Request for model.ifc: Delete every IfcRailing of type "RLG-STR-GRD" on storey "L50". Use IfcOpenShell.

First a look at what the model holds.

```python
import ifcopenshell
import ifcopenshell.util.element

model = ifcopenshell.open("model.ifc")
print(model.schema)
storey = next(s for s in model.by_type("IfcBuildingStorey") if s.Name == "L50")
railings = [e for e in ifcopenshell.util.element.get_decomposition(storey) if e.is_a("IfcRailing")]
seen = {}
for e in railings:
    element_type = ifcopenshell.util.element.get_type(e)
    name = element_type.Name if element_type not in (None, e) else None
    seen[name] = seen.get(name, 0) + 1
for name, count in sorted(seen.items(), key=str):
    print(count, "x", name)
```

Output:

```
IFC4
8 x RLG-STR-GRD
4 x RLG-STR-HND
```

```python
import ifcopenshell
import ifcopenshell.api.root
import ifcopenshell.util.element

model = ifcopenshell.open("model.ifc")

storey = next(s for s in model.by_type("IfcBuildingStorey") if s.Name == "L50")
railings = [e for e in ifcopenshell.util.element.get_decomposition(storey) if e.is_a("IfcRailing")]
targets = [e for e in railings if (t := ifcopenshell.util.element.get_type(e)) not in (None, e) and t.Name == "RLG-STR-GRD"]

for e in targets:
    ifcopenshell.api.root.remove_product(model, product=e)
print(len(targets), "removed")

model.write("model_v2.ifc")
```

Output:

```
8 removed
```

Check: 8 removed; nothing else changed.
